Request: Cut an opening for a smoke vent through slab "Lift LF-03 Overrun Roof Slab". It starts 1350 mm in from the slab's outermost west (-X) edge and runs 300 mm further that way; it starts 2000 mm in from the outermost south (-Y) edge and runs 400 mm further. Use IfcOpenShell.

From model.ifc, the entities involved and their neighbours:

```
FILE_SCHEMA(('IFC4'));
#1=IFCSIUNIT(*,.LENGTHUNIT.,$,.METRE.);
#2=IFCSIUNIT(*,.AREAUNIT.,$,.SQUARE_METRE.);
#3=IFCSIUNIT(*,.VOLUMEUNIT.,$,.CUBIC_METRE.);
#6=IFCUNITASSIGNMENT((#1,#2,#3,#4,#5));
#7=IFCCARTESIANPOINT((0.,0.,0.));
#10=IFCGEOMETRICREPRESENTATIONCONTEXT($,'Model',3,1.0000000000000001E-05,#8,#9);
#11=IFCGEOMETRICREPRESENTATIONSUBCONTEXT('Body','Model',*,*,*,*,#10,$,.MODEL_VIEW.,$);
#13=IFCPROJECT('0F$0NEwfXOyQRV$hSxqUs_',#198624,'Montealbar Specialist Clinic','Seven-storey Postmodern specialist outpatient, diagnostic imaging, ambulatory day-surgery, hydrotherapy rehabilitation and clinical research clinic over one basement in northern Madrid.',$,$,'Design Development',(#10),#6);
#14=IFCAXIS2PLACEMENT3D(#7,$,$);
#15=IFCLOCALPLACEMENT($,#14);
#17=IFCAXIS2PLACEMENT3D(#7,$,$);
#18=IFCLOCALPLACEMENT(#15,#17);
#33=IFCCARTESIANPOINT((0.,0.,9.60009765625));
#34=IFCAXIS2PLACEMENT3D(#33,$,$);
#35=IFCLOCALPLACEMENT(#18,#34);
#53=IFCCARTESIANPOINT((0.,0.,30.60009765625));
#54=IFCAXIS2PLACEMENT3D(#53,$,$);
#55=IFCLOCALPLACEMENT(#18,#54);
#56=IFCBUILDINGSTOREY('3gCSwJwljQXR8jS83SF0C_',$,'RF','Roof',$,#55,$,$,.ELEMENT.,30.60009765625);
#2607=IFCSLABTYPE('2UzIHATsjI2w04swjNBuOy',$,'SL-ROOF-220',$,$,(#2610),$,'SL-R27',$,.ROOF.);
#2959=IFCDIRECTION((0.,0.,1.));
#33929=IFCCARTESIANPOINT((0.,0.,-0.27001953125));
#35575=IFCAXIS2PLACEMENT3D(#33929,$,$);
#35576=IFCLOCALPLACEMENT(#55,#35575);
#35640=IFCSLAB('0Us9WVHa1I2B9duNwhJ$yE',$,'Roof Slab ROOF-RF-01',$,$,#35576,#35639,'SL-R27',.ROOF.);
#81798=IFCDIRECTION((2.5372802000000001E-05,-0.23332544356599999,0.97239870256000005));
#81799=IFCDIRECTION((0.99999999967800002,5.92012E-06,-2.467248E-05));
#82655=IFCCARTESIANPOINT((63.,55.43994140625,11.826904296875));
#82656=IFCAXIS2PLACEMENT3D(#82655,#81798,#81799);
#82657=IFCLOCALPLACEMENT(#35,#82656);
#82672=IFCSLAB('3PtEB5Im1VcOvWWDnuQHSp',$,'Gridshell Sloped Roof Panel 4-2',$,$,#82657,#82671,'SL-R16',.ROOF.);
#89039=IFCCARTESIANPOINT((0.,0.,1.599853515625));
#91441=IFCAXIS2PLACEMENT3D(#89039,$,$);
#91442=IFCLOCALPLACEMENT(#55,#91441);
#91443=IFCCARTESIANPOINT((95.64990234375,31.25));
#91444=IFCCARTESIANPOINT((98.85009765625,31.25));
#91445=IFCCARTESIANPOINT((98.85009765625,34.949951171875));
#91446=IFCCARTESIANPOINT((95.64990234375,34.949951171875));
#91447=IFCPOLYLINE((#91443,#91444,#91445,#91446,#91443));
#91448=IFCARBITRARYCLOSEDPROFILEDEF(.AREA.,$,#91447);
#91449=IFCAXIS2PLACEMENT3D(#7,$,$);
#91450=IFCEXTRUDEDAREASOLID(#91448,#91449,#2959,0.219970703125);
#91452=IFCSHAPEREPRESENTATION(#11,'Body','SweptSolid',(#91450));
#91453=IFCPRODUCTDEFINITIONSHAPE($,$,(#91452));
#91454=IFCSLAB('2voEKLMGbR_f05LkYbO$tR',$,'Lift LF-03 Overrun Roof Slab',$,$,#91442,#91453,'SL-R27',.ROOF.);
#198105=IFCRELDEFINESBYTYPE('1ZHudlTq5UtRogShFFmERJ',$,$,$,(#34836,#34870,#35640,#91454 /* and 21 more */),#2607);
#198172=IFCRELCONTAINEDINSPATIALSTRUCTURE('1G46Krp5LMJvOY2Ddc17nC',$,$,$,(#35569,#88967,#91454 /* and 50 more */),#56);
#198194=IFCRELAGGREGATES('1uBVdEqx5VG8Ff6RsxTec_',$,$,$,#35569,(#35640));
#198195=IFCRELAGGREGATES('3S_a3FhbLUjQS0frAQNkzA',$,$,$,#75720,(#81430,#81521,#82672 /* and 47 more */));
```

```python
import numpy as np
import ifcopenshell
import ifcopenshell.api.feature
import ifcopenshell.api.geometry
import ifcopenshell.api.root
import ifcopenshell.geom
import ifcopenshell.util.placement
import ifcopenshell.util.representation
import ifcopenshell.util.shape
import ifcopenshell.util.unit

model = ifcopenshell.open("model.ifc")
unit_scale = ifcopenshell.util.unit.calculate_unit_scale(model)
settings = ifcopenshell.geom.settings()


def volume(element):
    """Net volume in cubic metres, openings subtracted."""
    shape = ifcopenshell.geom.create_shape(settings, element)
    return ifcopenshell.util.shape.get_volume(shape.geometry)


slab = model.by_guid("2voEKLMGbR_f05LkYbO$tR")
before = volume(slab)

# Extent in the slab's own axes, in metres. The edges named are its -X and -Y sides.
slab_shape = ifcopenshell.geom.create_shape(settings, slab)
vertices = ifcopenshell.util.shape.get_vertices(slab_shape.geometry)
x_min, y_min, bottom = vertices.min(axis=0)
top = vertices[:, 2].max()

opening = ifcopenshell.api.root.create_entity(model, ifc_class="IfcOpeningElement", name="Smoke vent opening", predefined_type="OPENING")
context = ifcopenshell.util.representation.get_context(model, "Model", "Body", "MODEL_VIEW")
width, depth = 0.3, 0.4
outline = [(0.0, 0.0), (width, 0.0), (width, depth), (0.0, depth), (0.0, 0.0)]
# Overshoot both faces by 50 mm so the cut is clean.
shape = ifcopenshell.api.geometry.add_slab_representation(
    model, context=context, depth=top - bottom + 0.1, polyline=outline
)
ifcopenshell.api.geometry.assign_representation(model, product=opening, representation=shape)

matrix = ifcopenshell.util.placement.get_local_placement(slab.ObjectPlacement)
matrix[:, 3] = matrix @ np.append(np.array([x_min + 1.35, y_min + 2, bottom - 0.05]) / unit_scale, 1.0)
ifcopenshell.api.geometry.edit_object_placement(model, product=opening, matrix=matrix, is_si=False)
ifcopenshell.api.feature.add_feature(model, feature=opening, element=slab)

after = volume(slab)

print(f"slab volume {before:.3f} -> {after:.3f} m3")

model.write("model_edited.ifc")
```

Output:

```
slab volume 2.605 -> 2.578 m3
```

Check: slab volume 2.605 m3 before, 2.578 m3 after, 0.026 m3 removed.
